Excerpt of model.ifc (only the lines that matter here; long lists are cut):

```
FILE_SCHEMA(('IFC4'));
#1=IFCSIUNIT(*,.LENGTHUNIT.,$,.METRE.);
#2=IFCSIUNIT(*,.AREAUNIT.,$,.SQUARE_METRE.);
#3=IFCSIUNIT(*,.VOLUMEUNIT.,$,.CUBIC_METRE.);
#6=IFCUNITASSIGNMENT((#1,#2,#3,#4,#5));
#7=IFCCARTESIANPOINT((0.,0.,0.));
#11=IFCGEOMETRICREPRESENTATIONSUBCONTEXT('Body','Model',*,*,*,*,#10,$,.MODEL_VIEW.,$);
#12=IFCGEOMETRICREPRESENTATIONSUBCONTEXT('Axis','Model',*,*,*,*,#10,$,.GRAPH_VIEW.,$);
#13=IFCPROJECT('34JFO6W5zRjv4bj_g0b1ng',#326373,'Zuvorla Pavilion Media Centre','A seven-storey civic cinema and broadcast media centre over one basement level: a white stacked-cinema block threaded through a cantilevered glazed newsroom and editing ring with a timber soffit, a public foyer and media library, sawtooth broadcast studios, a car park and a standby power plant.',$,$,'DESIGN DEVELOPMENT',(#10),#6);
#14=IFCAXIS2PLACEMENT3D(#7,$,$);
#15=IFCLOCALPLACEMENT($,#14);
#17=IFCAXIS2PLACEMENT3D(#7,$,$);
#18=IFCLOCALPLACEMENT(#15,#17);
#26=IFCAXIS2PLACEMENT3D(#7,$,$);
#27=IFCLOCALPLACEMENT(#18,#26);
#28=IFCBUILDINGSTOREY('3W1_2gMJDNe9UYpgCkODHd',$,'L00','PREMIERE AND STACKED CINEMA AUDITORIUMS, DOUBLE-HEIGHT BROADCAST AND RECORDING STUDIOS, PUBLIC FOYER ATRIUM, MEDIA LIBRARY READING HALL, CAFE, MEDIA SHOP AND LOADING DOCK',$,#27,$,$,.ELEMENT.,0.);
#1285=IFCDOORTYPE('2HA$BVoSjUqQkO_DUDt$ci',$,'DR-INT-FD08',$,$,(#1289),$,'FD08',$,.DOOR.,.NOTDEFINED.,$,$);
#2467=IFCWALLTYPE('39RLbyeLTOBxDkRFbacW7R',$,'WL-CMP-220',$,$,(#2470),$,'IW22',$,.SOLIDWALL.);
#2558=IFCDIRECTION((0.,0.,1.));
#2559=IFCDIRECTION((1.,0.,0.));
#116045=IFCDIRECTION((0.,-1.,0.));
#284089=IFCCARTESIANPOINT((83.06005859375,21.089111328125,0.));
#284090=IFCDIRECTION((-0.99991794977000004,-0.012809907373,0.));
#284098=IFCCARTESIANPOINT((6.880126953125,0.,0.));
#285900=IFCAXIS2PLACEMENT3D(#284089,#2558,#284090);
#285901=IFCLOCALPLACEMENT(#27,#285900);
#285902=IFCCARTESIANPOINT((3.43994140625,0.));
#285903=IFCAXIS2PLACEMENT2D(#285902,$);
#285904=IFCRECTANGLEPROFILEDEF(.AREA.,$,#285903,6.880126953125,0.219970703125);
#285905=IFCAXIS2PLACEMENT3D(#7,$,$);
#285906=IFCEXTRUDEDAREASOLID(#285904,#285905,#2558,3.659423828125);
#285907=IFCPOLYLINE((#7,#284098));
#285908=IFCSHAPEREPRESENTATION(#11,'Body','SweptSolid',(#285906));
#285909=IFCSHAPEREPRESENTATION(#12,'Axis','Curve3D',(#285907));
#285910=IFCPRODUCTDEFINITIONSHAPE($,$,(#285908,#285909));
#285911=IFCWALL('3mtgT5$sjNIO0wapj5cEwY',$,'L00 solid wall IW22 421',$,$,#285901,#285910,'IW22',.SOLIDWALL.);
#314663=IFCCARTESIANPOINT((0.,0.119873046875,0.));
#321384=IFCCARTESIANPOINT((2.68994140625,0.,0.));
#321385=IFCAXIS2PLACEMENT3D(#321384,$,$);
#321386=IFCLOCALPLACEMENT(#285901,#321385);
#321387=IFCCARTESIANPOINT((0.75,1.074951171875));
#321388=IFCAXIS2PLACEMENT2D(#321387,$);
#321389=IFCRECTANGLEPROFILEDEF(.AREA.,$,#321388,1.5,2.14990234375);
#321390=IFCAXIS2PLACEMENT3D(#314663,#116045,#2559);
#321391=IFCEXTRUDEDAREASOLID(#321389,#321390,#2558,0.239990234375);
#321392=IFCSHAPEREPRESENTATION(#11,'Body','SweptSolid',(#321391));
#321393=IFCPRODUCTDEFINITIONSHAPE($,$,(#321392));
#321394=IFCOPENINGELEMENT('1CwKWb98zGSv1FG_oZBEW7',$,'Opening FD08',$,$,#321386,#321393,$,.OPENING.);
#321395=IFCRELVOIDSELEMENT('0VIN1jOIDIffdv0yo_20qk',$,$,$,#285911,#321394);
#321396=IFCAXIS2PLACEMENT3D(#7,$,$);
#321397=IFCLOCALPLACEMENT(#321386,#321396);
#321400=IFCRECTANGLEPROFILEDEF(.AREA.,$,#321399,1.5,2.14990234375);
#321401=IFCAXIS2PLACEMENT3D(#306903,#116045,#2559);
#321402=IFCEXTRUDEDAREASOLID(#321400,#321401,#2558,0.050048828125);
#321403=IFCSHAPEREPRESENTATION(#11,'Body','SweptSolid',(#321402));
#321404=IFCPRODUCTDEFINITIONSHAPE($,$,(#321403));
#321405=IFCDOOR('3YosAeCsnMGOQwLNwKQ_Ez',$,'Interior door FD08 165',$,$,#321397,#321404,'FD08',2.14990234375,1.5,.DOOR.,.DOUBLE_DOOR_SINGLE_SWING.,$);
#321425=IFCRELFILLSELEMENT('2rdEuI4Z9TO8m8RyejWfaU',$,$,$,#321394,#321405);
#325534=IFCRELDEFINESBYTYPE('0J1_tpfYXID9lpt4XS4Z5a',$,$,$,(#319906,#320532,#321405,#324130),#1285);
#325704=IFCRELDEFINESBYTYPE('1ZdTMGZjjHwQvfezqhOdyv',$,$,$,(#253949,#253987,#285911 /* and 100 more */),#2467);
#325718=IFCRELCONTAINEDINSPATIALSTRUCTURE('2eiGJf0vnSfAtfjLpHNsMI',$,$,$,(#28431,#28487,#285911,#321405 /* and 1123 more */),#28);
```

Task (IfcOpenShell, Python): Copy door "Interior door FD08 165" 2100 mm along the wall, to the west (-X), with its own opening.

```python
import ifcopenshell
import ifcopenshell.api.feature
import ifcopenshell.api.geometry
import ifcopenshell.api.root
import ifcopenshell.geom
import ifcopenshell.util.element
import ifcopenshell.util.placement
import ifcopenshell.util.shape

model = ifcopenshell.open("model.ifc")
settings = ifcopenshell.geom.settings()


def volume(element):
    """Net volume in cubic metres, openings subtracted."""
    shape = ifcopenshell.geom.create_shape(settings, element)
    return ifcopenshell.util.shape.get_volume(shape.geometry)


door = model.by_guid("3YosAeCsnMGOQwLNwKQ_Ez")
opening = door.FillsVoids[0].RelatingOpeningElement
wall = opening.VoidsElements[0].RelatingBuildingElement
before = volume(wall)
shift = ifcopenshell.util.placement.get_local_placement(wall.ObjectPlacement)[:3, 0] * 2.1

# copy_class copies the void relationship, type, container and properties, but no geometry.
new_opening = ifcopenshell.api.root.copy_class(model, product=opening)
new_opening.Representation = ifcopenshell.util.element.copy_deep(
    model, opening.Representation, exclude=["IfcGeometricRepresentationContext", "IfcRepresentationMap"]
)
new_door = ifcopenshell.api.root.copy_class(model, product=door)
new_door.Representation = ifcopenshell.util.element.copy_deep(
    model, door.Representation, exclude=["IfcGeometricRepresentationContext", "IfcRepresentationMap"]
)
new_door.Tag = None
ifcopenshell.api.feature.add_filling(model, opening=new_opening, element=new_door)

for old, new in ((opening, new_opening), (door, new_door)):
    matrix = ifcopenshell.util.placement.get_local_placement(old.ObjectPlacement)
    matrix[:3, 3] += shift
    ifcopenshell.api.geometry.edit_object_placement(model, product=new, matrix=matrix, is_si=False)

after = volume(wall)

print(f"wall volume {before:.3f} -> {after:.3f} m3")

model.write("model_v2.ifc")
```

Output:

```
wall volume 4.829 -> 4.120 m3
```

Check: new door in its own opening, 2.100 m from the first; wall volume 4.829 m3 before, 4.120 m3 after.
